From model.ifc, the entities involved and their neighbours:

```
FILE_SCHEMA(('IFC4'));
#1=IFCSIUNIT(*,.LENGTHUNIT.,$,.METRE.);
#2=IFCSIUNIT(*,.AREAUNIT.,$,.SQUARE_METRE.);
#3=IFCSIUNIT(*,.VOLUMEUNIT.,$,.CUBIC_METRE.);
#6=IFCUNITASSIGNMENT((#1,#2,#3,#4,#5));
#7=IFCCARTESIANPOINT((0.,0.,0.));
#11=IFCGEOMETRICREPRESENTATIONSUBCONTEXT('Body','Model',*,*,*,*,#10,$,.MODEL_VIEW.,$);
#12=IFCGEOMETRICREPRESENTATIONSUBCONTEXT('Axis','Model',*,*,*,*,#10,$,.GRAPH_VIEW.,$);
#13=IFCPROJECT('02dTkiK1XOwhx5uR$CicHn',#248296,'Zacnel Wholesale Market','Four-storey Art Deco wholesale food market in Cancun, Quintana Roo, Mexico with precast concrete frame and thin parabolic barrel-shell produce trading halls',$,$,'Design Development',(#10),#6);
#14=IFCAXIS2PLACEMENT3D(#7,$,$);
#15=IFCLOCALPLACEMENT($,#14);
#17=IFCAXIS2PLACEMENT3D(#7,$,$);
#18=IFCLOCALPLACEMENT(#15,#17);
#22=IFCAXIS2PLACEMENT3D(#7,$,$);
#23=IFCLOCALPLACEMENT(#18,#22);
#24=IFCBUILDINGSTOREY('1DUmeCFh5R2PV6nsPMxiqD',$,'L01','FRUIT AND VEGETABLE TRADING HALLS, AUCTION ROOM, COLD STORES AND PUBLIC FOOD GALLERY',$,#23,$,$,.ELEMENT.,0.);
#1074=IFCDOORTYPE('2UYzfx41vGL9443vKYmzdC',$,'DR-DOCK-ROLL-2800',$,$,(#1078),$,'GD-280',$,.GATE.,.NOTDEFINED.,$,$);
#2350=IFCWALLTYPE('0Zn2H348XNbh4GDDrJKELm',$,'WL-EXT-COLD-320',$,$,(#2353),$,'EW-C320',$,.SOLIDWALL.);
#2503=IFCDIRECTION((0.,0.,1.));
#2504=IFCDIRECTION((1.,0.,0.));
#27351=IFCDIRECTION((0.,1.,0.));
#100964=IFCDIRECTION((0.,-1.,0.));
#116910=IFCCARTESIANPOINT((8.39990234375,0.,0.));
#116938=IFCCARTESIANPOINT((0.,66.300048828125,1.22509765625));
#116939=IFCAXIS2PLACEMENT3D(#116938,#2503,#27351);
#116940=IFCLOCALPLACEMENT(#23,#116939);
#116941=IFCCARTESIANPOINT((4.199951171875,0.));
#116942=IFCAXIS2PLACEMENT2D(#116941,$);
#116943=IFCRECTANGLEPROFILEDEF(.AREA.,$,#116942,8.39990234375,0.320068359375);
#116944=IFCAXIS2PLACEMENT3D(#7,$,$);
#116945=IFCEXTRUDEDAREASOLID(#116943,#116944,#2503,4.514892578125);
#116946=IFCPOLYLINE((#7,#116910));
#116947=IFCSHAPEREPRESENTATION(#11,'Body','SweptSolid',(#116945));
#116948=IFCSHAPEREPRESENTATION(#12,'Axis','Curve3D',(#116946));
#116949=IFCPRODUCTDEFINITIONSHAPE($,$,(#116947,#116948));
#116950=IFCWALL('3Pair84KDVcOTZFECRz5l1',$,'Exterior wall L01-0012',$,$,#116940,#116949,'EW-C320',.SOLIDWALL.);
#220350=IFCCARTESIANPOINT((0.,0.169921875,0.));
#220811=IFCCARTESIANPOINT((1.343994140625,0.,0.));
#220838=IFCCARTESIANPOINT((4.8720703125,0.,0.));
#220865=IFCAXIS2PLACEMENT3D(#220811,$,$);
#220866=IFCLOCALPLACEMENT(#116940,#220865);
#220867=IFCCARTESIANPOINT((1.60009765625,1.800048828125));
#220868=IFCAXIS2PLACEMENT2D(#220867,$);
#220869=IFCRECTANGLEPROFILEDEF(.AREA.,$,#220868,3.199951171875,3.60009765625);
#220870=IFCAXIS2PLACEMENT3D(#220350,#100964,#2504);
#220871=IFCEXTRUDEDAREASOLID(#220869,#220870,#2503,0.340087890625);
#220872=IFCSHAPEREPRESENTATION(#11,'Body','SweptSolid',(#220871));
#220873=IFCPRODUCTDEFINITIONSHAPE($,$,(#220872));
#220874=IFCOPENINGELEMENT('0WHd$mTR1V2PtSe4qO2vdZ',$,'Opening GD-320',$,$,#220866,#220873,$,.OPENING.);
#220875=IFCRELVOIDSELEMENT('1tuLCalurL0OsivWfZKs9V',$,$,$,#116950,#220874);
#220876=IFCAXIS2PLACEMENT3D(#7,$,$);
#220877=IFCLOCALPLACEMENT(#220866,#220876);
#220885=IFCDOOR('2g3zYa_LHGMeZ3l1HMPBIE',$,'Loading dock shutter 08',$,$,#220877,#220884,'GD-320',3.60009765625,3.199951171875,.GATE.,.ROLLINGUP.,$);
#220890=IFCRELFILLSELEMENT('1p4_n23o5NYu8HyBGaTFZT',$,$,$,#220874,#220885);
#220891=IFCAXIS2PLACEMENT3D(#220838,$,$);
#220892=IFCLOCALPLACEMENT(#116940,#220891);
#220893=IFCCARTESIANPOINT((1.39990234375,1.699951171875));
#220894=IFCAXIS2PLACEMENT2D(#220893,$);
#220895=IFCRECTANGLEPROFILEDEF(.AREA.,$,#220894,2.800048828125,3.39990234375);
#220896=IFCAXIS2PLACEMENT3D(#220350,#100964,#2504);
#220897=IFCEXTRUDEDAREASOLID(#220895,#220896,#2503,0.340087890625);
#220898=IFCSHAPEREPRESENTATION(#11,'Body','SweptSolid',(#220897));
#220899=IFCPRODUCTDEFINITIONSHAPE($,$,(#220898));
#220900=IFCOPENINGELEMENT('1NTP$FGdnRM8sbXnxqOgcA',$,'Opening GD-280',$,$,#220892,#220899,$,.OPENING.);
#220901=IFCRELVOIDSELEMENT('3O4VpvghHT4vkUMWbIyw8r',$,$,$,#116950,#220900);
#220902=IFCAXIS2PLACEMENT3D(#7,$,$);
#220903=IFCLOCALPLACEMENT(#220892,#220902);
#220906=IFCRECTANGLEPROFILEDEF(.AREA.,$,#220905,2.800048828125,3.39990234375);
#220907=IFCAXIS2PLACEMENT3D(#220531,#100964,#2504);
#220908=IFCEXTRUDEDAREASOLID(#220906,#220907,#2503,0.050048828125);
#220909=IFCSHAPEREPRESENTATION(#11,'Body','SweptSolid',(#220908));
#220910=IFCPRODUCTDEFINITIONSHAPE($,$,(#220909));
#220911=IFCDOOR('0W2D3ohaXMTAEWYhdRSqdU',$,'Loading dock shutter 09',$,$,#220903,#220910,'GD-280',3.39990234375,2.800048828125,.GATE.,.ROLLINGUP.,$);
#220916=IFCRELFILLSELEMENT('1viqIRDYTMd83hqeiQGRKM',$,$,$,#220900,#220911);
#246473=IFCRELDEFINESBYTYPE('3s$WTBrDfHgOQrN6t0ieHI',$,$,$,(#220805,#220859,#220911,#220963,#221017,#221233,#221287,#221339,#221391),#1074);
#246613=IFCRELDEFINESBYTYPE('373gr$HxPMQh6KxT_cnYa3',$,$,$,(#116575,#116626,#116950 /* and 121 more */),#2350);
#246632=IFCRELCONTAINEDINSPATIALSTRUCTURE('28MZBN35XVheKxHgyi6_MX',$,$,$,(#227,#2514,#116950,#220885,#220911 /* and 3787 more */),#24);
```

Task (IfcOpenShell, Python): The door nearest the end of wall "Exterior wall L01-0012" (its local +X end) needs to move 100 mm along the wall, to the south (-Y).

```python
import ifcopenshell
import ifcopenshell.api.geometry
import ifcopenshell.util.placement

model = ifcopenshell.open("model.ifc")

door = model.by_id(220911)
opening = door.FillsVoids[0].RelatingOpeningElement
wall = opening.VoidsElements[0].RelatingBuildingElement

wall_matrix = ifcopenshell.util.placement.get_local_placement(wall.ObjectPlacement)
shift = wall_matrix[:3, 0] * -0.1
before = ifcopenshell.util.placement.get_local_placement(door.ObjectPlacement)[:3, 3].copy()

# The door is placed relative to its opening, so it follows when the opening moves.
matrix = ifcopenshell.util.placement.get_local_placement(opening.ObjectPlacement)
matrix[:3, 3] += shift
ifcopenshell.api.geometry.edit_object_placement(
    model, product=opening, matrix=matrix, is_si=False, should_transform_children=True
)

after = ifcopenshell.util.placement.get_local_placement(door.ObjectPlacement)[:3, 3]
print("door moved by", (after - before).round(3) + 0.0)

model.write("model_v2.ifc")
```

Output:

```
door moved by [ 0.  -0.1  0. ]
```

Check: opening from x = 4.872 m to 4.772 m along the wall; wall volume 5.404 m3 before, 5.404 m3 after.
